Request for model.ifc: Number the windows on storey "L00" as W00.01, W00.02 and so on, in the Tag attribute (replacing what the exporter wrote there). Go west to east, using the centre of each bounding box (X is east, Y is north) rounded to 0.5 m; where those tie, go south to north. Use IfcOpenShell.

First a look at what the model holds.

```python
import ifcopenshell
import ifcopenshell.util.element
import ifcopenshell.util.placement

model = ifcopenshell.open("model.ifc")
print(model.schema)
storey = next(s for s in model.by_type("IfcBuildingStorey") if s.Name == "L00")
windows = [e for e in ifcopenshell.util.element.get_decomposition(storey) if e.is_a("IfcWindow")]
for e in sorted(windows, key=lambda e: e.id()):
    origin = ifcopenshell.util.placement.get_local_placement(e.ObjectPlacement)[:3, 3]
    print(e.id(), e.Tag, e.Name, origin.round(2) + 0.0, sep=" | ")
```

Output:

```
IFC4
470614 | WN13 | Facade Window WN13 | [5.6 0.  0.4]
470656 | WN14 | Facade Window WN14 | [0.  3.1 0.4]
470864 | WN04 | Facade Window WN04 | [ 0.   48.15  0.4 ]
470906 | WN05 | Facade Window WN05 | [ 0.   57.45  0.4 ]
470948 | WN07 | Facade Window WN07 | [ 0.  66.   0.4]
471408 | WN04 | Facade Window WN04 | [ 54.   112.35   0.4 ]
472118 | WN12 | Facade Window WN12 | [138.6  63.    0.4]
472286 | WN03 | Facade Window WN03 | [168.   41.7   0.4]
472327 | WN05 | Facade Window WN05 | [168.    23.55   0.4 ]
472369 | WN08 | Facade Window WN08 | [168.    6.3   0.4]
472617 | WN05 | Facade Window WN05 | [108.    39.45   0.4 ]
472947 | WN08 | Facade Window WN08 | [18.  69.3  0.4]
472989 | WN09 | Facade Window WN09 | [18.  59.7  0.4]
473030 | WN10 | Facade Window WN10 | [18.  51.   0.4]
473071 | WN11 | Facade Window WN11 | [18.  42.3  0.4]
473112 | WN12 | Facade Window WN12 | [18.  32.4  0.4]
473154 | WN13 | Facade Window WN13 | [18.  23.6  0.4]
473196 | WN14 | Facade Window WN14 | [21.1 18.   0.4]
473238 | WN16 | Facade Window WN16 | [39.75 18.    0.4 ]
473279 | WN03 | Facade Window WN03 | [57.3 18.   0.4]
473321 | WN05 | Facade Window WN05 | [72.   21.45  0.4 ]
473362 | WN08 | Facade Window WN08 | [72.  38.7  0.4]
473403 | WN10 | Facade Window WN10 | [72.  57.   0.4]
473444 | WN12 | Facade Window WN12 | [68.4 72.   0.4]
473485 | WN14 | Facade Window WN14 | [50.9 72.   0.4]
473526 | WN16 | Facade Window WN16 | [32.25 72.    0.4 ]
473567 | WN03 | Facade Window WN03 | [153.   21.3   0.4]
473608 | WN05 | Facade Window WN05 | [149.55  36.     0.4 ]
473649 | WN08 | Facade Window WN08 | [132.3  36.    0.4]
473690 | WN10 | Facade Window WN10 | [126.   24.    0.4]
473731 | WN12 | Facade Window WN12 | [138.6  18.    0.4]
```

```python
import ifcopenshell
import ifcopenshell.geom
import ifcopenshell.util.element
import ifcopenshell.util.shape

model = ifcopenshell.open("model.ifc")
settings = ifcopenshell.geom.settings()
settings.set("use-world-coords", True)


def centre(element):
    shape = ifcopenshell.geom.create_shape(settings, element)
    return ifcopenshell.util.shape.get_bbox_centroid(shape.geometry)


storey = next(s for s in model.by_type("IfcBuildingStorey") if s.Name == "L00")
windows = [e for e in ifcopenshell.util.element.get_decomposition(storey) if e.is_a("IfcWindow")]

# Insertion points can sit at a corner or the storey origin, so sort by the geometry (in metres).
centres = {e: centre(e) for e in windows}
windows.sort(key=lambda e: (round(centres[e][0] / 0.5), centres[e][1]))

for i, e in enumerate(windows, start=1):
    number = f"W00.{i:02d}"
    e.Tag = number
    print(e.id(), number)

model.write("model_edited.ifc")
```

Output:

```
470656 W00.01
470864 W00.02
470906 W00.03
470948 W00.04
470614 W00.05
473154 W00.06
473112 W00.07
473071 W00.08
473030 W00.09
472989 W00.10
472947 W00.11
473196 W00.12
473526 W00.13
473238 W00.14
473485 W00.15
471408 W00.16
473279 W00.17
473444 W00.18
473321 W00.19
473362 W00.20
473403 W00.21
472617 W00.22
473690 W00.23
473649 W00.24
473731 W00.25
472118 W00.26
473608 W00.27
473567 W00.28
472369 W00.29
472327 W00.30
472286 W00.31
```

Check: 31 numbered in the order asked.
